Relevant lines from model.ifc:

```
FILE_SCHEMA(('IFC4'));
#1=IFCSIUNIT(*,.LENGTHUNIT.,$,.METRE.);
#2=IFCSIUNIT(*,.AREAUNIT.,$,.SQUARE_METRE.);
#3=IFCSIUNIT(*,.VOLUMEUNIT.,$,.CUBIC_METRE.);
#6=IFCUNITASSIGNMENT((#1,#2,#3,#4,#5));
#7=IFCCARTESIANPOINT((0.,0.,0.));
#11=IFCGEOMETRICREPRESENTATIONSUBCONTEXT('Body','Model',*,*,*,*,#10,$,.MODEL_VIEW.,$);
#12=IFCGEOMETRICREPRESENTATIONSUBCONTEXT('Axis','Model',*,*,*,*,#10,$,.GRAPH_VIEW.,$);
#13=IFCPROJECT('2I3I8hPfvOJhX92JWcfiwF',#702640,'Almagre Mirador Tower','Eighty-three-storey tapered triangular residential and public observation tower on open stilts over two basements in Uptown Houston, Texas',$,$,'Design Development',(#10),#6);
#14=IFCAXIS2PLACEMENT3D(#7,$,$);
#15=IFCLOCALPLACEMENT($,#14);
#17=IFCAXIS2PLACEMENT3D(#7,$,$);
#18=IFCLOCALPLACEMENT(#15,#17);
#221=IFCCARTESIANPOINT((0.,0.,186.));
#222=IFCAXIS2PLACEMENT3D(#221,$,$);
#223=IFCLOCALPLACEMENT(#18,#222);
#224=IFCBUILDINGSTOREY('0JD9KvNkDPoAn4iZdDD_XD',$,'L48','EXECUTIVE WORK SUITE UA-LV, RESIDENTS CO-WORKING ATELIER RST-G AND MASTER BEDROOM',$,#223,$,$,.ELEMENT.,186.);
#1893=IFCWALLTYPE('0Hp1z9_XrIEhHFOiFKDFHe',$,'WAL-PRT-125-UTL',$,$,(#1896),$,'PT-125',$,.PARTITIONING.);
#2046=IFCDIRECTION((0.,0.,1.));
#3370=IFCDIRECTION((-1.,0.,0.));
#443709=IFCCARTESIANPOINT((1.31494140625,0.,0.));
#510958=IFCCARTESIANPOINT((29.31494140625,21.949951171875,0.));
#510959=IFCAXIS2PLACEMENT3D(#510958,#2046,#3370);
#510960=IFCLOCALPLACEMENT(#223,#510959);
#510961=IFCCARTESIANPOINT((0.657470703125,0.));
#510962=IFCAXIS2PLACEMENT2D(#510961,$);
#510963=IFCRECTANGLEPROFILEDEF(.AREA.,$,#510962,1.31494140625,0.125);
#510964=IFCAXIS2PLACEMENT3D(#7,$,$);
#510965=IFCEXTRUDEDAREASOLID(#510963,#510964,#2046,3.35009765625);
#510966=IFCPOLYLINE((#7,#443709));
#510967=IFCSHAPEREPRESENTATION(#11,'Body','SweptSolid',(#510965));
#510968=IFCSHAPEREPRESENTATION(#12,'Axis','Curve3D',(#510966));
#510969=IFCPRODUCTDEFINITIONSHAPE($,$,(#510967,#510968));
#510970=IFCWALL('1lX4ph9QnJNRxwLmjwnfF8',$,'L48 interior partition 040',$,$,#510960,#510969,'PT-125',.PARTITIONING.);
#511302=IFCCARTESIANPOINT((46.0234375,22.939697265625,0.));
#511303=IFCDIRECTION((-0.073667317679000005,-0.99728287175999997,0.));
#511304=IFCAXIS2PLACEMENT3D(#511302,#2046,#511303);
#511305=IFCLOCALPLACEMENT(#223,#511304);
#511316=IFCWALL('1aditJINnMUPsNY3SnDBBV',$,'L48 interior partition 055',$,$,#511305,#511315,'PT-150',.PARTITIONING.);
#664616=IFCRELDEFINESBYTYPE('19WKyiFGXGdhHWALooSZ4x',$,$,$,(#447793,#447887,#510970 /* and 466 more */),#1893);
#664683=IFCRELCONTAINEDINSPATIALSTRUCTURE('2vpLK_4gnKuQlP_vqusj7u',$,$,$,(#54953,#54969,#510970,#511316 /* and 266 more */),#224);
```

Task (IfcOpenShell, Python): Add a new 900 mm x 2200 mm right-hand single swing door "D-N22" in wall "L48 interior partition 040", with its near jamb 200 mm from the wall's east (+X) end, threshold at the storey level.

```python
import numpy as np
import ifcopenshell
import ifcopenshell.api.feature
import ifcopenshell.api.geometry
import ifcopenshell.api.root
import ifcopenshell.api.spatial
import ifcopenshell.geom
import ifcopenshell.util.element
import ifcopenshell.util.placement
import ifcopenshell.util.representation
import ifcopenshell.util.shape
import ifcopenshell.util.unit

model = ifcopenshell.open("model.ifc")
unit_scale = ifcopenshell.util.unit.calculate_unit_scale(model)
settings = ifcopenshell.geom.settings()


def volume(element):
    """Net volume in cubic metres, openings subtracted."""
    shape = ifcopenshell.geom.create_shape(settings, element)
    return ifcopenshell.util.shape.get_volume(shape.geometry)


wall = model.by_guid("1lX4ph9QnJNRxwLmjwnfF8")
storey = ifcopenshell.util.element.get_container(wall, ifc_class="IfcBuildingStorey")
context = ifcopenshell.util.representation.get_context(model, "Model", "Body", "MODEL_VIEW")
before = volume(wall)

width, height, from_end, sill = 0.9, 2.2, 0.2, 0.0  # metres

# The wall runs along its own X axis, and the end named is its -X end.
wall_shape = ifcopenshell.geom.create_shape(settings, wall)
x, y, z = ifcopenshell.util.shape.get_vertices(wall_shape.geometry).T
start = x.min() + from_end
face, thickness = float(y.min()), float(y.max() - y.min())
wall_matrix = ifcopenshell.util.placement.get_local_placement(wall.ObjectPlacement)
level = ifcopenshell.util.placement.get_local_placement(storey.ObjectPlacement)[2, 3]


def in_wall(x, y):
    """Placement at x, y metres in the wall's axes, at sill height."""
    matrix = wall_matrix.copy()
    matrix[:, 3] = wall_matrix @ np.array([x / unit_scale, y / unit_scale, 0.0, 1.0])
    matrix[2, 3] = level + sill / unit_scale
    return matrix


# Opening: a box that overshoots both wall faces by 50 mm.
opening = ifcopenshell.api.root.create_entity(model, ifc_class="IfcOpeningElement", predefined_type="OPENING")
box = ifcopenshell.api.geometry.add_wall_representation(
    model, context=context, length=width, height=height, thickness=thickness + 0.1
)
ifcopenshell.api.geometry.assign_representation(model, product=opening, representation=box)
ifcopenshell.api.geometry.edit_object_placement(model, product=opening, matrix=in_wall(start, face - 0.05), is_si=False)
ifcopenshell.api.feature.add_feature(model, feature=opening, element=wall)

door = ifcopenshell.api.root.create_entity(model, ifc_class="IfcDoor", name="D-N22", predefined_type="DOOR")
door.OverallWidth, door.OverallHeight = width / unit_scale, height / unit_scale
door.OperationType = "SINGLE_SWING_RIGHT"
body = ifcopenshell.api.geometry.add_door_representation(
    model,
    context=context,
    overall_width=door.OverallWidth,
    overall_height=door.OverallHeight,
    operation_type="SINGLE_SWING_RIGHT",
    lining_properties={"LiningDepth": thickness / unit_scale, "ThresholdDepth": thickness / unit_scale},
)
ifcopenshell.api.geometry.assign_representation(model, product=door, representation=body)
ifcopenshell.api.spatial.assign_container(model, products=[door], relating_structure=storey)
ifcopenshell.api.feature.add_filling(model, opening=opening, element=door)

# The lining spans the wall, so the door starts at the wall face.
ifcopenshell.api.geometry.edit_object_placement(model, product=door, matrix=in_wall(start, face), is_si=False)

after = volume(wall)

print(f"wall volume {before:.3f} -> {after:.3f} m3")

model.write("model_rev.ifc")
```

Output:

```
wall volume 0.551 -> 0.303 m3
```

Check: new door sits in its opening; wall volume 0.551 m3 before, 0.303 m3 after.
